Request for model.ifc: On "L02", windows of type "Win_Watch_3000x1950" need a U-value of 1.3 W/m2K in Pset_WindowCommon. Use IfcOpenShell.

First a look at what the model holds.

```python
import ifcopenshell
import ifcopenshell.util.element

model = ifcopenshell.open("model.ifc")
print(model.schema)
storey = next(s for s in model.by_type("IfcBuildingStorey") if s.Name == "L02")
windows = [e for e in ifcopenshell.util.element.get_decomposition(storey) if e.is_a("IfcWindow")]
seen = {}
for e in windows:
    element_type = ifcopenshell.util.element.get_type(e)
    key = (element_type.Name if element_type != e and element_type else None, ifcopenshell.util.element.get_pset(e, "Pset_WindowCommon", "ThermalTransmittance"))
    seen[key] = seen.get(key, 0) + 1
for (name, value), count in sorted(seen.items(), key=str):
    print(count, "x", name, "|", value)
```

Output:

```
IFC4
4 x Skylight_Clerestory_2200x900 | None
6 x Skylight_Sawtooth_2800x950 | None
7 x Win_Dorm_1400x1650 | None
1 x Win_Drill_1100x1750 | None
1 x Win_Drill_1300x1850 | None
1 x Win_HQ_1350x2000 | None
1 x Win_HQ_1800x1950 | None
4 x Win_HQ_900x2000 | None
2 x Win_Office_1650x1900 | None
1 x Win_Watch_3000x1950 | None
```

```python
import ifcopenshell
import ifcopenshell.api.pset
import ifcopenshell.util.element

model = ifcopenshell.open("model.ifc")

storey = next(s for s in model.by_type("IfcBuildingStorey") if s.Name == "L02")
windows = [e for e in ifcopenshell.util.element.get_decomposition(storey) if e.is_a("IfcWindow")]

count = 0
for e in windows:
    element_type = ifcopenshell.util.element.get_type(e)
    if element_type in (None, e) or element_type.Name != "Win_Watch_3000x1950":
        continue
    # add_pset returns the element's existing set when there is one.
    pset = ifcopenshell.api.pset.add_pset(model, product=e, name="Pset_WindowCommon")
    ifcopenshell.api.pset.edit_pset(model, pset=pset, properties={"ThermalTransmittance": 1.3})
    count += 1

print(count, "windows updated")

model.write("model_edited.ifc")
```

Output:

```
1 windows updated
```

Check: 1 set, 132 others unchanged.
